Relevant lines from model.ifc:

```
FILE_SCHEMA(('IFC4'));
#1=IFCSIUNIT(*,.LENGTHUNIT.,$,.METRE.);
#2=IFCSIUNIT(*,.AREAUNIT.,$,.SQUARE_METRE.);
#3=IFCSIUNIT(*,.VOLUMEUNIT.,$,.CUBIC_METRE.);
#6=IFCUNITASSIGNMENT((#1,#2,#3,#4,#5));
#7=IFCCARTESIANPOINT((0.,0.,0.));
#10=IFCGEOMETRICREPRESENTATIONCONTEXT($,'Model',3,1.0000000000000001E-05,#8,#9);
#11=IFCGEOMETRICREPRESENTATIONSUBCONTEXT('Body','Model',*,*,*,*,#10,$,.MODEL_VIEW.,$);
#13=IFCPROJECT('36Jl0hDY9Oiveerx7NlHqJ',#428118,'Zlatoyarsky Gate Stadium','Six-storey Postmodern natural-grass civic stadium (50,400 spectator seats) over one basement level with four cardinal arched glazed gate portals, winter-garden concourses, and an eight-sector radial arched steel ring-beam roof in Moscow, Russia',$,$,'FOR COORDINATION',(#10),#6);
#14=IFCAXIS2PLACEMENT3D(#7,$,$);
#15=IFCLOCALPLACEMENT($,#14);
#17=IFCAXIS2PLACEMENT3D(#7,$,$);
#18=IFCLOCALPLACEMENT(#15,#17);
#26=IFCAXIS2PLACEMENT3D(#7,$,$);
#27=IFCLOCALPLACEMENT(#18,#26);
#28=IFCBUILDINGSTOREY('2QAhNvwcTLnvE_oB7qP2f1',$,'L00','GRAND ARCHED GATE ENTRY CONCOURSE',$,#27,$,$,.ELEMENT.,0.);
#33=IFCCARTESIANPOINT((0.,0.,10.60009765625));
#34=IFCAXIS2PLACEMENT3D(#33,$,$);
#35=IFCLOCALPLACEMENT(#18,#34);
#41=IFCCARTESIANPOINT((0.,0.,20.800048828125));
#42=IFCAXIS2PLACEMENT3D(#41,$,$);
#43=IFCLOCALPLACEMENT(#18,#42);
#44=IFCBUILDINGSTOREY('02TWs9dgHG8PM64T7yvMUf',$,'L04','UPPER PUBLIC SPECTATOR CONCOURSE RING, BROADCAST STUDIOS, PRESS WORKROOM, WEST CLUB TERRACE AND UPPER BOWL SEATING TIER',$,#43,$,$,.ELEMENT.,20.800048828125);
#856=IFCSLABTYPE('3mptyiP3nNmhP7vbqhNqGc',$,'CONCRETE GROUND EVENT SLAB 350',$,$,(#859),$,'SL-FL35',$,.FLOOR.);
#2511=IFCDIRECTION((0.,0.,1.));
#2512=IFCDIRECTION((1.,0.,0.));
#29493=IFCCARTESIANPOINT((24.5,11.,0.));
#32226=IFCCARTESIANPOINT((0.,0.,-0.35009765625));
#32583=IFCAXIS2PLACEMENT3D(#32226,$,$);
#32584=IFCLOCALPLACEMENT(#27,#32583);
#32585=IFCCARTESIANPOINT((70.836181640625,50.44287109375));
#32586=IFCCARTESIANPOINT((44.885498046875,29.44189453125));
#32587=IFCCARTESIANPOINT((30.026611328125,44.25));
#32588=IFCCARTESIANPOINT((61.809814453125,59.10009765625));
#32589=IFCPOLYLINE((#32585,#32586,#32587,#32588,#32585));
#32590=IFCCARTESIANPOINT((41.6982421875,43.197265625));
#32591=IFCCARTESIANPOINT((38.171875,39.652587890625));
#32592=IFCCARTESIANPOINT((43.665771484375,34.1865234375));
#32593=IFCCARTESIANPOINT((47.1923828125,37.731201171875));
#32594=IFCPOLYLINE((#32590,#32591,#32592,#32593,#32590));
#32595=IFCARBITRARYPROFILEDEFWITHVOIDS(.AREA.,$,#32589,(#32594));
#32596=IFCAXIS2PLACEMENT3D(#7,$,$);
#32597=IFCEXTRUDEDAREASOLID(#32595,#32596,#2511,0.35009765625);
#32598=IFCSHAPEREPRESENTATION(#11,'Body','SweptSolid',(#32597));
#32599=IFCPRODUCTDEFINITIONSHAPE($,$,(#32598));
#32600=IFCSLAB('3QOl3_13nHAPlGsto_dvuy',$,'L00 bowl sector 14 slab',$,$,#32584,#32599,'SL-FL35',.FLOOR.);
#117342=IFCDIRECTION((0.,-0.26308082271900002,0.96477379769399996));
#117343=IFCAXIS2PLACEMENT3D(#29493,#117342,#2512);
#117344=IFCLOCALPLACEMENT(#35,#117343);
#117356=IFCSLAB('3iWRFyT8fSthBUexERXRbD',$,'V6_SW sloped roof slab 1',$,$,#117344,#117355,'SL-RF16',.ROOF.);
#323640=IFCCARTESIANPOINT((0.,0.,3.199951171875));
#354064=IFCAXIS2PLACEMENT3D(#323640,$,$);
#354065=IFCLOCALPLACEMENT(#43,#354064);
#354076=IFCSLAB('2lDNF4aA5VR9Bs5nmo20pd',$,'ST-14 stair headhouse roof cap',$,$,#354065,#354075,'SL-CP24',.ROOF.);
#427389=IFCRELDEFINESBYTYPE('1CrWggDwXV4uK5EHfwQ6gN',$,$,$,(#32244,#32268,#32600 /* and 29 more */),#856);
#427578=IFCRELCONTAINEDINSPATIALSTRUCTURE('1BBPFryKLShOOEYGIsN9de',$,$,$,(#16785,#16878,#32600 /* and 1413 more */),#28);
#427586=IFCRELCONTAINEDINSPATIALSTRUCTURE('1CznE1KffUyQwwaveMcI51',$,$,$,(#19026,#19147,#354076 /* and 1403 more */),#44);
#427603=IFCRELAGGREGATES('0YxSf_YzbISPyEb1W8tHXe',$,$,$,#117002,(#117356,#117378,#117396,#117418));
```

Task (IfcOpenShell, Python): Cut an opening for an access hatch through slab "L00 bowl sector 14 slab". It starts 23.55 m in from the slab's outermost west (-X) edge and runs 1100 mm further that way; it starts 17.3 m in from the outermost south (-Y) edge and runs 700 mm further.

```python
import numpy as np
import ifcopenshell
import ifcopenshell.api.feature
import ifcopenshell.api.geometry
import ifcopenshell.api.root
import ifcopenshell.geom
import ifcopenshell.util.placement
import ifcopenshell.util.representation
import ifcopenshell.util.shape
import ifcopenshell.util.unit

model = ifcopenshell.open("model.ifc")
unit_scale = ifcopenshell.util.unit.calculate_unit_scale(model)
settings = ifcopenshell.geom.settings()


def volume(element):
    """Net volume in cubic metres, openings subtracted."""
    shape = ifcopenshell.geom.create_shape(settings, element)
    return ifcopenshell.util.shape.get_volume(shape.geometry)


slab = model.by_id(32600)
before = volume(slab)

# Extent in the slab's own axes, in metres. The edges named are its -X and -Y sides.
slab_shape = ifcopenshell.geom.create_shape(settings, slab)
vertices = ifcopenshell.util.shape.get_vertices(slab_shape.geometry)
x_min, y_min, bottom = vertices.min(axis=0)
top = vertices[:, 2].max()

opening = ifcopenshell.api.root.create_entity(model, ifc_class="IfcOpeningElement", name="Access hatch opening", predefined_type="OPENING")
context = ifcopenshell.util.representation.get_context(model, "Model", "Body", "MODEL_VIEW")
width, depth = 1.1, 0.7
outline = [(0.0, 0.0), (width, 0.0), (width, depth), (0.0, depth), (0.0, 0.0)]
# Overshoot both faces by 50 mm so the cut is clean.
shape = ifcopenshell.api.geometry.add_slab_representation(
    model, context=context, depth=top - bottom + 0.1, polyline=outline
)
ifcopenshell.api.geometry.assign_representation(model, product=opening, representation=shape)

matrix = ifcopenshell.util.placement.get_local_placement(slab.ObjectPlacement)
matrix[:, 3] = matrix @ np.append(np.array([x_min + 23.55, y_min + 17.3, bottom - 0.05]) / unit_scale, 1.0)
ifcopenshell.api.geometry.edit_object_placement(model, product=opening, matrix=matrix, is_si=False)
ifcopenshell.api.feature.add_feature(model, feature=opening, element=slab)

after = volume(slab)

print(f"slab volume {before:.3f} -> {after:.3f} m3")

model.write("model_rev.ifc")
```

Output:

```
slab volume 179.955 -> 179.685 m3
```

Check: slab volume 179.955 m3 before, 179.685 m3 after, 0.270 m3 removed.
